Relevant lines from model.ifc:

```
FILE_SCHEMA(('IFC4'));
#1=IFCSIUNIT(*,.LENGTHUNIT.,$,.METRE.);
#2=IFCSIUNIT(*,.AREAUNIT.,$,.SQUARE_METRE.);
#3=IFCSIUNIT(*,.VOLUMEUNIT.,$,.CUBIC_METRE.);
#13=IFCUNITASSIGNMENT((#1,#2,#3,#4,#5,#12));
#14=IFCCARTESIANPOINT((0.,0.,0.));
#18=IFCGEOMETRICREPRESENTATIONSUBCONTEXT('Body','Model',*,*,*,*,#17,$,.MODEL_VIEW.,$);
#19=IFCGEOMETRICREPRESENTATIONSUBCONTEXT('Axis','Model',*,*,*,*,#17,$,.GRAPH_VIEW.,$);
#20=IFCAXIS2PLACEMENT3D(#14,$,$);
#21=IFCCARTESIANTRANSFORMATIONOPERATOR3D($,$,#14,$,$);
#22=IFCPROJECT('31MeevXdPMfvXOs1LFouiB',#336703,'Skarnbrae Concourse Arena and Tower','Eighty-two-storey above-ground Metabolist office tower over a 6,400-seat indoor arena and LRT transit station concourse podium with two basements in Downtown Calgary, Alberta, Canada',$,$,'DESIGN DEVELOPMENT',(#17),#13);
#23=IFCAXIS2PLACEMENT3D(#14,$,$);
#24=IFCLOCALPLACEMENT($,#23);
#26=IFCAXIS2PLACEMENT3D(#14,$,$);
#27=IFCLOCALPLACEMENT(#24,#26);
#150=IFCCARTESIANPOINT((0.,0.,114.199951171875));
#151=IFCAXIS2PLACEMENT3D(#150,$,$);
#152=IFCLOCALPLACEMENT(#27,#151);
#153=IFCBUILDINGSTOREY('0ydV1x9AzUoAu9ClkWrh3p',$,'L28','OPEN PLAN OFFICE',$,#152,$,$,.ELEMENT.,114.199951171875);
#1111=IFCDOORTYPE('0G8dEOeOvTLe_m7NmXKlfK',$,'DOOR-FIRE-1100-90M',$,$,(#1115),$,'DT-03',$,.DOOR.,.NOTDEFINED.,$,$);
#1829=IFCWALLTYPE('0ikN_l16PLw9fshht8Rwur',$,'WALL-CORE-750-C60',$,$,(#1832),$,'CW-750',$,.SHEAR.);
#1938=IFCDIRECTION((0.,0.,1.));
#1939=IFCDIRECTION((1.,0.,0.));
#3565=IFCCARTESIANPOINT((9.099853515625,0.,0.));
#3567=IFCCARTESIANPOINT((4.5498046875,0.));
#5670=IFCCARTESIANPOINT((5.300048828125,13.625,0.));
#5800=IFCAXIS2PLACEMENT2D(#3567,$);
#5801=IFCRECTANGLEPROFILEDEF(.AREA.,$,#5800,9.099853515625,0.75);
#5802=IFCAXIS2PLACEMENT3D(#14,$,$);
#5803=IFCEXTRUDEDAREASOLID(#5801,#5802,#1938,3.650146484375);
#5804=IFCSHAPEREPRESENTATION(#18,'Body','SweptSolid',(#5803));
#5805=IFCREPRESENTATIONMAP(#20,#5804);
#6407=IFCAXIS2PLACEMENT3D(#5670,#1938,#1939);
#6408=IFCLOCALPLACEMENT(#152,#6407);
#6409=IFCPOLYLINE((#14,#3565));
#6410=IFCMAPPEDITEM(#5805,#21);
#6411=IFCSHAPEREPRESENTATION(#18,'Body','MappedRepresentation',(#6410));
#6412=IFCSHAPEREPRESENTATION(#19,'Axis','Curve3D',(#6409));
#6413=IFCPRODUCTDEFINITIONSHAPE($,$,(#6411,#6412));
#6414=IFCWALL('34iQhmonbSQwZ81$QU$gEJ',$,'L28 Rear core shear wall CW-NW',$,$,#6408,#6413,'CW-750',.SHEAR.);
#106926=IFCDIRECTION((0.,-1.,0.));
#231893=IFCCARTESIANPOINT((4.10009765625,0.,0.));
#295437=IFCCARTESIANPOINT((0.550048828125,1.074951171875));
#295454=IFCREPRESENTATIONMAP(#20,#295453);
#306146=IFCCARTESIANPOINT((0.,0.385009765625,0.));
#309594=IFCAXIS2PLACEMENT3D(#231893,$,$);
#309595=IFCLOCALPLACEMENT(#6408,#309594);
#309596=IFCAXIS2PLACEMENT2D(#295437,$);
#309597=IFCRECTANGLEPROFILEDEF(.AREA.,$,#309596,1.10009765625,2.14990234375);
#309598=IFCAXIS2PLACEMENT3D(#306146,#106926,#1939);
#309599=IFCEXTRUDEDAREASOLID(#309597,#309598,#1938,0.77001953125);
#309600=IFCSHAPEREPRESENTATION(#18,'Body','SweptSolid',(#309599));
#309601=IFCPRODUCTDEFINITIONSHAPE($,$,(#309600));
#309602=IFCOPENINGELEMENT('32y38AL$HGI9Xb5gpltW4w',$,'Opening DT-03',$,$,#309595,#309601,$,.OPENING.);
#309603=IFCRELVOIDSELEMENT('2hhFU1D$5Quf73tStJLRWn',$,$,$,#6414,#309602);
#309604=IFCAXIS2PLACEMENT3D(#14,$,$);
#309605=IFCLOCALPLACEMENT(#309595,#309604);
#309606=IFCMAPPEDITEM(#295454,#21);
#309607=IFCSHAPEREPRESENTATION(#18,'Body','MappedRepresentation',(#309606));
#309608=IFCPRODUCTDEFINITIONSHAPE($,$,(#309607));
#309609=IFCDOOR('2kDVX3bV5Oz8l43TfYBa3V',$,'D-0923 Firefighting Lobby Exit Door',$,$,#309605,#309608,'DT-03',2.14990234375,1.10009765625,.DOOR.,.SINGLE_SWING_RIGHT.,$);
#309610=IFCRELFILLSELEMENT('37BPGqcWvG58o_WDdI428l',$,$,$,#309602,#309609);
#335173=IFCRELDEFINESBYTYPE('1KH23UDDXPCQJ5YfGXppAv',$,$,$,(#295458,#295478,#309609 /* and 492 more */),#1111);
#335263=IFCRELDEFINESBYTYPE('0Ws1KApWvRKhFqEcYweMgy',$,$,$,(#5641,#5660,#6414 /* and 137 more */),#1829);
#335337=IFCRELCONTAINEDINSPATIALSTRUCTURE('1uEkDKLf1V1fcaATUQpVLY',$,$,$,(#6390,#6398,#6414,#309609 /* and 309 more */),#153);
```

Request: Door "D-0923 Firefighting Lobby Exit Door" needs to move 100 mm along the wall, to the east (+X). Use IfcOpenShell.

```python
import ifcopenshell
import ifcopenshell.api.geometry
import ifcopenshell.util.placement

model = ifcopenshell.open("model.ifc")

door = model.by_id(309609)
opening = door.FillsVoids[0].RelatingOpeningElement
wall = opening.VoidsElements[0].RelatingBuildingElement

wall_matrix = ifcopenshell.util.placement.get_local_placement(wall.ObjectPlacement)
shift = wall_matrix[:3, 0] * 0.1
before = ifcopenshell.util.placement.get_local_placement(door.ObjectPlacement)[:3, 3].copy()

# The door is placed relative to its opening, so it follows when the opening moves.
matrix = ifcopenshell.util.placement.get_local_placement(opening.ObjectPlacement)
matrix[:3, 3] += shift
ifcopenshell.api.geometry.edit_object_placement(
    model, product=opening, matrix=matrix, is_si=False, should_transform_children=True
)

after = ifcopenshell.util.placement.get_local_placement(door.ObjectPlacement)[:3, 3]
print("door moved by", (after - before).round(3) + 0.0)

model.write("model_v2.ifc")
```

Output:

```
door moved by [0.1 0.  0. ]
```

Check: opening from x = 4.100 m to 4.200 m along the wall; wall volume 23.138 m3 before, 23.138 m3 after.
